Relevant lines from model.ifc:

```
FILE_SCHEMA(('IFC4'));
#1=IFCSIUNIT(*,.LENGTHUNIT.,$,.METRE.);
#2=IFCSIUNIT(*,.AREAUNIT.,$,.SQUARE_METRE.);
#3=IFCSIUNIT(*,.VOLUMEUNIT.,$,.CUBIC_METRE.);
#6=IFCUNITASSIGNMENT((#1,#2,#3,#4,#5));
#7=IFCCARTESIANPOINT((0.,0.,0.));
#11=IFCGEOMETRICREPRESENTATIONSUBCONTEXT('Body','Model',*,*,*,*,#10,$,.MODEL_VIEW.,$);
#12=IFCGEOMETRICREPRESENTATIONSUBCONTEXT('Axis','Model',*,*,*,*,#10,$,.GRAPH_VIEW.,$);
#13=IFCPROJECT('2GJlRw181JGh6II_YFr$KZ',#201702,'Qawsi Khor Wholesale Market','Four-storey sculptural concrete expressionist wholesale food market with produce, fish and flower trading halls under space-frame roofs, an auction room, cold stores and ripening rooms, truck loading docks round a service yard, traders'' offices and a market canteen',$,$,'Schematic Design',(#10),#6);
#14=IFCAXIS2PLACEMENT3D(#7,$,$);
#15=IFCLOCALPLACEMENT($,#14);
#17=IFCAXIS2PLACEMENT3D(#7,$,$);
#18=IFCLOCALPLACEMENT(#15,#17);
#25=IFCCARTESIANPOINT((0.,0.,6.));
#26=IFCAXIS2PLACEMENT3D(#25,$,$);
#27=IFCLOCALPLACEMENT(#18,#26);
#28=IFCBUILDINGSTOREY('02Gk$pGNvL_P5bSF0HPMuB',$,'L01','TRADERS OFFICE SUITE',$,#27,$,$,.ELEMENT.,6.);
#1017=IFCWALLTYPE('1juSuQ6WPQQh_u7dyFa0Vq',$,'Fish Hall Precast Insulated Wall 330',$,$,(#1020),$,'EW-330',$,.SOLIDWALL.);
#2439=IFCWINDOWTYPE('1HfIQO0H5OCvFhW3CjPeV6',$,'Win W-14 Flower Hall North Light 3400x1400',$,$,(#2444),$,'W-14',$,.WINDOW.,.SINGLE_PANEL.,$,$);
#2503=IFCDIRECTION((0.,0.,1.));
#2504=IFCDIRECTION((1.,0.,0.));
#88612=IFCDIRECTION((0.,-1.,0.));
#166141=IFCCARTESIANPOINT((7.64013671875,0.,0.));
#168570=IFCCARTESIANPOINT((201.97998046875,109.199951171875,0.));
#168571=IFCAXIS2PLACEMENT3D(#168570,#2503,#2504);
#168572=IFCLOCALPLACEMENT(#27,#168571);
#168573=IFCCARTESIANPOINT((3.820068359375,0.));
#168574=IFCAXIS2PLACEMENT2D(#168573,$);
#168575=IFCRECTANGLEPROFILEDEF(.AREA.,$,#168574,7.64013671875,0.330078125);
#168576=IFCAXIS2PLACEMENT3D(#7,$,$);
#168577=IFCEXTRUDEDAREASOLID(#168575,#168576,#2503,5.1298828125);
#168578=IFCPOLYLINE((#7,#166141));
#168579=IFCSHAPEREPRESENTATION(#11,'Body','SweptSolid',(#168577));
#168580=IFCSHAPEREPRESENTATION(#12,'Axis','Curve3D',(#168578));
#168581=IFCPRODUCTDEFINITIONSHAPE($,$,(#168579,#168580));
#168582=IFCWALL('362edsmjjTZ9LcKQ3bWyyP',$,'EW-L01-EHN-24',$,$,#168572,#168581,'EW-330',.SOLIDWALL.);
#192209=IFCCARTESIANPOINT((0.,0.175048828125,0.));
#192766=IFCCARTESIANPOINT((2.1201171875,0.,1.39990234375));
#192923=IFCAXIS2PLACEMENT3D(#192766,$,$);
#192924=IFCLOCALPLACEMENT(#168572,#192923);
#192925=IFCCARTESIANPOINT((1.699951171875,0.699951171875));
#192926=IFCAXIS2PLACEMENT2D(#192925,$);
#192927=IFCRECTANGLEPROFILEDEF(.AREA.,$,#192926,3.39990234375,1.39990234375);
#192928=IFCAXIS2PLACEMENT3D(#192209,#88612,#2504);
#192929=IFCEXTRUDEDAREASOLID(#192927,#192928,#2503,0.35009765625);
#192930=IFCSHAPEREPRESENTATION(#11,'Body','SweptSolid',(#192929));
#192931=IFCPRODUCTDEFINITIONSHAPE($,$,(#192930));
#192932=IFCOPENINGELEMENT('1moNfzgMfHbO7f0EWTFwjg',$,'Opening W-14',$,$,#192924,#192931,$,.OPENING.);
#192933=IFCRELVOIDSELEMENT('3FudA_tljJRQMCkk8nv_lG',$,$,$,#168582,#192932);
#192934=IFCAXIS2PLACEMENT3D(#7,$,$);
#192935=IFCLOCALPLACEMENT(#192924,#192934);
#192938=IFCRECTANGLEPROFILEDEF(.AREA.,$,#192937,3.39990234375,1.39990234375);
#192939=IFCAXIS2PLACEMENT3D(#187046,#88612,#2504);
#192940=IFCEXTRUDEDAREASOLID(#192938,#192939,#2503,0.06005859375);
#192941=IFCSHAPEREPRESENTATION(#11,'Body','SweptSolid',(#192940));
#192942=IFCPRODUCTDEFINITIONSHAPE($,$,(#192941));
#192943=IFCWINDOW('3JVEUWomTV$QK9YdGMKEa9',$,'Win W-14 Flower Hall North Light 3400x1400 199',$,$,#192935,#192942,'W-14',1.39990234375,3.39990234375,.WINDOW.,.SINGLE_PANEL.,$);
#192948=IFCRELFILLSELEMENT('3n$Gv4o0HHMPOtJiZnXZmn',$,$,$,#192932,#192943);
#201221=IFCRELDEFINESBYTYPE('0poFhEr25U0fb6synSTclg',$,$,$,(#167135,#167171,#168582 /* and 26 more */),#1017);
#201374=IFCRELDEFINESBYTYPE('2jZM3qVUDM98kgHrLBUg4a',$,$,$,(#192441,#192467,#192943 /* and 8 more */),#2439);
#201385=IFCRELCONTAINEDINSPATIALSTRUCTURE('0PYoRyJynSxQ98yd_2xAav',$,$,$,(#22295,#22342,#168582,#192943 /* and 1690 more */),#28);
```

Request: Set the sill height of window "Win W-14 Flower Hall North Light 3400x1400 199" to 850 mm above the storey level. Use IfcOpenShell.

```python
import numpy as np
import ifcopenshell
import ifcopenshell.api.geometry
import ifcopenshell.geom
import ifcopenshell.util.element
import ifcopenshell.util.placement
import ifcopenshell.util.shape
import ifcopenshell.util.unit

model = ifcopenshell.open("model.ifc")
unit_scale = ifcopenshell.util.unit.calculate_unit_scale(model)

window = model.by_guid("3JVEUWomTV$QK9YdGMKEa9")
opening = window.FillsVoids[0].RelatingOpeningElement
storey = ifcopenshell.util.element.get_container(window, ifc_class="IfcBuildingStorey")
level = ifcopenshell.util.placement.get_local_placement(storey.ObjectPlacement)[2, 3]

# The opening's origin need not be at the sill, so measure its lowest point.
shape = ifcopenshell.geom.create_shape(ifcopenshell.geom.settings(), opening)
bottom = ifcopenshell.util.shape.get_shape_bottom_elevation(shape, shape.geometry) / unit_scale
dz = level + 0.85 / unit_scale - bottom

shift = np.array([0.0, 0.0, dz])
# The window is placed relative to its opening, so it follows when the opening moves.
matrix = ifcopenshell.util.placement.get_local_placement(opening.ObjectPlacement)
matrix[:3, 3] += shift
ifcopenshell.api.geometry.edit_object_placement(
    model, product=opening, matrix=matrix, is_si=False, should_transform_children=True
)

print(f"moved by {dz * unit_scale:+.3f} m")

model.write("model_v2.ifc")
```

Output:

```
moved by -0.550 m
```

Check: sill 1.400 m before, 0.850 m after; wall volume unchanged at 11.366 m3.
